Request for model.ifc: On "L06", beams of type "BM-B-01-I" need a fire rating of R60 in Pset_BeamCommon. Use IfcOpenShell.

First a look at what the model holds.

```python
import ifcopenshell
import ifcopenshell.util.element

model = ifcopenshell.open("model.ifc")
print(model.schema)
storey = next(s for s in model.by_type("IfcBuildingStorey") if s.Name == "L06")
beams = [e for e in ifcopenshell.util.element.get_decomposition(storey) if e.is_a("IfcBeam")]
seen = {}
for e in beams:
    element_type = ifcopenshell.util.element.get_type(e)
    key = (element_type.Name if element_type != e and element_type else None, ifcopenshell.util.element.get_pset(e, "Pset_BeamCommon", "FireRating"))
    seen[key] = seen.get(key, 0) + 1
for (name, value), count in sorted(seen.items(), key=str):
    print(count, "x", name, "|", value)
```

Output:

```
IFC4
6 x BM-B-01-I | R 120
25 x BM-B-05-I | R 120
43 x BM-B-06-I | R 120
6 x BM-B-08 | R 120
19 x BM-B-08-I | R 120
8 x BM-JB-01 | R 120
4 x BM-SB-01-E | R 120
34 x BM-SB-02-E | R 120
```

```python
import ifcopenshell
import ifcopenshell.api.pset
import ifcopenshell.util.element

model = ifcopenshell.open("model.ifc")

storey = next(s for s in model.by_type("IfcBuildingStorey") if s.Name == "L06")
beams = [e for e in ifcopenshell.util.element.get_decomposition(storey) if e.is_a("IfcBeam")]

count = 0
for e in beams:
    element_type = ifcopenshell.util.element.get_type(e)
    if element_type in (None, e) or element_type.Name != "BM-B-01-I":
        continue
    # add_pset returns the element's existing set when there is one.
    pset = ifcopenshell.api.pset.add_pset(model, product=e, name="Pset_BeamCommon")
    ifcopenshell.api.pset.edit_pset(model, pset=pset, properties={"FireRating": "R60"})
    count += 1

print(count, "beams updated")

model.write("model_rev.ifc")
```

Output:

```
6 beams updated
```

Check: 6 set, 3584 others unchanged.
